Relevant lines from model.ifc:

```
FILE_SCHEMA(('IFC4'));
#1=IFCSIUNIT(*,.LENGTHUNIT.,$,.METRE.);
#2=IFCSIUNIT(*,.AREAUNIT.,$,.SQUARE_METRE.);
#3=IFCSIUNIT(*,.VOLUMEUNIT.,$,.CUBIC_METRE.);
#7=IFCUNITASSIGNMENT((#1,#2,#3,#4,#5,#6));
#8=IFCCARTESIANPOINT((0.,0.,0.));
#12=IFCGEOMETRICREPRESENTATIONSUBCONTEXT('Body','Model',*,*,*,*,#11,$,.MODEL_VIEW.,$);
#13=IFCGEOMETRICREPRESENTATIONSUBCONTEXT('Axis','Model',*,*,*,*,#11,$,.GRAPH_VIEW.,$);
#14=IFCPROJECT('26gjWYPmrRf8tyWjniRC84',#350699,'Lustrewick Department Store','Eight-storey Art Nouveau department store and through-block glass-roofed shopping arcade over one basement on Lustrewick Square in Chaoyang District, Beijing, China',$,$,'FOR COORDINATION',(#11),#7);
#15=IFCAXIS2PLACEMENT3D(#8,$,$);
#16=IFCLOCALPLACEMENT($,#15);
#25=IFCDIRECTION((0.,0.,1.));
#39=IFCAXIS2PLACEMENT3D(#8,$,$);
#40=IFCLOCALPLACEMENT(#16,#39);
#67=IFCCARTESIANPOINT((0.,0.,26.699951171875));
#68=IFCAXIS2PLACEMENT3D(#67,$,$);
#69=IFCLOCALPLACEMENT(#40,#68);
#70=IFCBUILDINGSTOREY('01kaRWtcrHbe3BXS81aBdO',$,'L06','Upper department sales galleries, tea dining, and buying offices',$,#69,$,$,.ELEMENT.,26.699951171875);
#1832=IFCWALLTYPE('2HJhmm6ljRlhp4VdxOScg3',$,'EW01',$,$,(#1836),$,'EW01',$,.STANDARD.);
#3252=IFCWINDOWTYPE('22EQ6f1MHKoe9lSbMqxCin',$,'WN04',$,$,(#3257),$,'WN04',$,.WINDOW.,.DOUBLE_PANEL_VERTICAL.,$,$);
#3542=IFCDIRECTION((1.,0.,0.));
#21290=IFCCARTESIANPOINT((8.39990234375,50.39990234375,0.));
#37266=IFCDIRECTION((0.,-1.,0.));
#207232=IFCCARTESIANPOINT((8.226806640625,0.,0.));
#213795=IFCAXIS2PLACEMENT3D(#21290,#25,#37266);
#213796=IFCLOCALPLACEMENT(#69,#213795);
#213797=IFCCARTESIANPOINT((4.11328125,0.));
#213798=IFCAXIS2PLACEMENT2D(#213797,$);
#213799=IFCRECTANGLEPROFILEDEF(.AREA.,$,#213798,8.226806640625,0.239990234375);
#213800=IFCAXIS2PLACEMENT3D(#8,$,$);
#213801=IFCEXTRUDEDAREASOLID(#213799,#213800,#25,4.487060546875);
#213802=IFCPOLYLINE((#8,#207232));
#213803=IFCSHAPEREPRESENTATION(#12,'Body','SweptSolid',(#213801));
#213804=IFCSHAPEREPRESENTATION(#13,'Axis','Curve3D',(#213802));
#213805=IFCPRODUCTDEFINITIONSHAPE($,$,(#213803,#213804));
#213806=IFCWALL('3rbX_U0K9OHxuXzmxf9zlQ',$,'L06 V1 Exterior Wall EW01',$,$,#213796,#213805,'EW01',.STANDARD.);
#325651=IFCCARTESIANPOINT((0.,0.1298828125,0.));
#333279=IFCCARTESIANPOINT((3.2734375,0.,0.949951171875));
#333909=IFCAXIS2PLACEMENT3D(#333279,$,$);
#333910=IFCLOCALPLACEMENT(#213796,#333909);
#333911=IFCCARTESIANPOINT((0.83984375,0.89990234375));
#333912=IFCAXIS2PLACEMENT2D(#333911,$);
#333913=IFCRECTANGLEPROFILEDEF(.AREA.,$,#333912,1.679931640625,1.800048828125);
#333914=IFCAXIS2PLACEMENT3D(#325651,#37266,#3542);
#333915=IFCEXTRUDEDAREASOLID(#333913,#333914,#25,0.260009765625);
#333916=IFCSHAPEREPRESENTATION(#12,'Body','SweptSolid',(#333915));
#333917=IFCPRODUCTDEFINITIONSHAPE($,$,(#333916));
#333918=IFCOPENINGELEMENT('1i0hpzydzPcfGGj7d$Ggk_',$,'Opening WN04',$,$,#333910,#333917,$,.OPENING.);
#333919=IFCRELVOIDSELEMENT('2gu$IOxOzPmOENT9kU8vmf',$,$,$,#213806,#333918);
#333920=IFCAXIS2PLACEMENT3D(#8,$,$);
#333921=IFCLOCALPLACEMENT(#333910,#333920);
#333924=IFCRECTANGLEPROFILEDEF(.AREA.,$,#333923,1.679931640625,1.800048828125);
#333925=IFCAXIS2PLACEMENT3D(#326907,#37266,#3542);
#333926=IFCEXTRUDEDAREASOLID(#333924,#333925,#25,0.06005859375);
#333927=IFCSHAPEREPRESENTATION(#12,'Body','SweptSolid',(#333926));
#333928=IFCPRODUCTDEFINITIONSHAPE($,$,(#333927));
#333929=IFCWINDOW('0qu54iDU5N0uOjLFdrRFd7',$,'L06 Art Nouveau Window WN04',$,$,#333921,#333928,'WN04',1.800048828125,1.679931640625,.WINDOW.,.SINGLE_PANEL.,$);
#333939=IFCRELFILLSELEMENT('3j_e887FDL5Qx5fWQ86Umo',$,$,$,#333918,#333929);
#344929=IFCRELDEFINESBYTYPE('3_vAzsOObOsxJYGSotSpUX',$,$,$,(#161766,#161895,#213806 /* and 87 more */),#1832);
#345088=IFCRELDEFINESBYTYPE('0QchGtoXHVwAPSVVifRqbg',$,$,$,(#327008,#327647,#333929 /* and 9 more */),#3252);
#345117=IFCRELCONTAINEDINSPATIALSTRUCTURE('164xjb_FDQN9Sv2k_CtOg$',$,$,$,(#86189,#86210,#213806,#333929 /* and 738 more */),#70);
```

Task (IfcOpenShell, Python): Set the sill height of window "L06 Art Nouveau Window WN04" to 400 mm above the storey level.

```python
import numpy as np
import ifcopenshell
import ifcopenshell.api.geometry
import ifcopenshell.geom
import ifcopenshell.util.element
import ifcopenshell.util.placement
import ifcopenshell.util.shape
import ifcopenshell.util.unit

model = ifcopenshell.open("model.ifc")
unit_scale = ifcopenshell.util.unit.calculate_unit_scale(model)

window = model.by_guid("0qu54iDU5N0uOjLFdrRFd7")
opening = window.FillsVoids[0].RelatingOpeningElement
storey = ifcopenshell.util.element.get_container(window, ifc_class="IfcBuildingStorey")
level = ifcopenshell.util.placement.get_local_placement(storey.ObjectPlacement)[2, 3]

# The opening's origin need not be at the sill, so measure its lowest point.
shape = ifcopenshell.geom.create_shape(ifcopenshell.geom.settings(), opening)
bottom = ifcopenshell.util.shape.get_shape_bottom_elevation(shape, shape.geometry) / unit_scale
dz = level + 0.4 / unit_scale - bottom

shift = np.array([0.0, 0.0, dz])
# The window is placed relative to its opening, so it follows when the opening moves.
matrix = ifcopenshell.util.placement.get_local_placement(opening.ObjectPlacement)
matrix[:3, 3] += shift
ifcopenshell.api.geometry.edit_object_placement(
    model, product=opening, matrix=matrix, is_si=False, should_transform_children=True
)

print(f"moved by {dz * unit_scale:+.3f} m")

model.write("model_edited.ifc")
```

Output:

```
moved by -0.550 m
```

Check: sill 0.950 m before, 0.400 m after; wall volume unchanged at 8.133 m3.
